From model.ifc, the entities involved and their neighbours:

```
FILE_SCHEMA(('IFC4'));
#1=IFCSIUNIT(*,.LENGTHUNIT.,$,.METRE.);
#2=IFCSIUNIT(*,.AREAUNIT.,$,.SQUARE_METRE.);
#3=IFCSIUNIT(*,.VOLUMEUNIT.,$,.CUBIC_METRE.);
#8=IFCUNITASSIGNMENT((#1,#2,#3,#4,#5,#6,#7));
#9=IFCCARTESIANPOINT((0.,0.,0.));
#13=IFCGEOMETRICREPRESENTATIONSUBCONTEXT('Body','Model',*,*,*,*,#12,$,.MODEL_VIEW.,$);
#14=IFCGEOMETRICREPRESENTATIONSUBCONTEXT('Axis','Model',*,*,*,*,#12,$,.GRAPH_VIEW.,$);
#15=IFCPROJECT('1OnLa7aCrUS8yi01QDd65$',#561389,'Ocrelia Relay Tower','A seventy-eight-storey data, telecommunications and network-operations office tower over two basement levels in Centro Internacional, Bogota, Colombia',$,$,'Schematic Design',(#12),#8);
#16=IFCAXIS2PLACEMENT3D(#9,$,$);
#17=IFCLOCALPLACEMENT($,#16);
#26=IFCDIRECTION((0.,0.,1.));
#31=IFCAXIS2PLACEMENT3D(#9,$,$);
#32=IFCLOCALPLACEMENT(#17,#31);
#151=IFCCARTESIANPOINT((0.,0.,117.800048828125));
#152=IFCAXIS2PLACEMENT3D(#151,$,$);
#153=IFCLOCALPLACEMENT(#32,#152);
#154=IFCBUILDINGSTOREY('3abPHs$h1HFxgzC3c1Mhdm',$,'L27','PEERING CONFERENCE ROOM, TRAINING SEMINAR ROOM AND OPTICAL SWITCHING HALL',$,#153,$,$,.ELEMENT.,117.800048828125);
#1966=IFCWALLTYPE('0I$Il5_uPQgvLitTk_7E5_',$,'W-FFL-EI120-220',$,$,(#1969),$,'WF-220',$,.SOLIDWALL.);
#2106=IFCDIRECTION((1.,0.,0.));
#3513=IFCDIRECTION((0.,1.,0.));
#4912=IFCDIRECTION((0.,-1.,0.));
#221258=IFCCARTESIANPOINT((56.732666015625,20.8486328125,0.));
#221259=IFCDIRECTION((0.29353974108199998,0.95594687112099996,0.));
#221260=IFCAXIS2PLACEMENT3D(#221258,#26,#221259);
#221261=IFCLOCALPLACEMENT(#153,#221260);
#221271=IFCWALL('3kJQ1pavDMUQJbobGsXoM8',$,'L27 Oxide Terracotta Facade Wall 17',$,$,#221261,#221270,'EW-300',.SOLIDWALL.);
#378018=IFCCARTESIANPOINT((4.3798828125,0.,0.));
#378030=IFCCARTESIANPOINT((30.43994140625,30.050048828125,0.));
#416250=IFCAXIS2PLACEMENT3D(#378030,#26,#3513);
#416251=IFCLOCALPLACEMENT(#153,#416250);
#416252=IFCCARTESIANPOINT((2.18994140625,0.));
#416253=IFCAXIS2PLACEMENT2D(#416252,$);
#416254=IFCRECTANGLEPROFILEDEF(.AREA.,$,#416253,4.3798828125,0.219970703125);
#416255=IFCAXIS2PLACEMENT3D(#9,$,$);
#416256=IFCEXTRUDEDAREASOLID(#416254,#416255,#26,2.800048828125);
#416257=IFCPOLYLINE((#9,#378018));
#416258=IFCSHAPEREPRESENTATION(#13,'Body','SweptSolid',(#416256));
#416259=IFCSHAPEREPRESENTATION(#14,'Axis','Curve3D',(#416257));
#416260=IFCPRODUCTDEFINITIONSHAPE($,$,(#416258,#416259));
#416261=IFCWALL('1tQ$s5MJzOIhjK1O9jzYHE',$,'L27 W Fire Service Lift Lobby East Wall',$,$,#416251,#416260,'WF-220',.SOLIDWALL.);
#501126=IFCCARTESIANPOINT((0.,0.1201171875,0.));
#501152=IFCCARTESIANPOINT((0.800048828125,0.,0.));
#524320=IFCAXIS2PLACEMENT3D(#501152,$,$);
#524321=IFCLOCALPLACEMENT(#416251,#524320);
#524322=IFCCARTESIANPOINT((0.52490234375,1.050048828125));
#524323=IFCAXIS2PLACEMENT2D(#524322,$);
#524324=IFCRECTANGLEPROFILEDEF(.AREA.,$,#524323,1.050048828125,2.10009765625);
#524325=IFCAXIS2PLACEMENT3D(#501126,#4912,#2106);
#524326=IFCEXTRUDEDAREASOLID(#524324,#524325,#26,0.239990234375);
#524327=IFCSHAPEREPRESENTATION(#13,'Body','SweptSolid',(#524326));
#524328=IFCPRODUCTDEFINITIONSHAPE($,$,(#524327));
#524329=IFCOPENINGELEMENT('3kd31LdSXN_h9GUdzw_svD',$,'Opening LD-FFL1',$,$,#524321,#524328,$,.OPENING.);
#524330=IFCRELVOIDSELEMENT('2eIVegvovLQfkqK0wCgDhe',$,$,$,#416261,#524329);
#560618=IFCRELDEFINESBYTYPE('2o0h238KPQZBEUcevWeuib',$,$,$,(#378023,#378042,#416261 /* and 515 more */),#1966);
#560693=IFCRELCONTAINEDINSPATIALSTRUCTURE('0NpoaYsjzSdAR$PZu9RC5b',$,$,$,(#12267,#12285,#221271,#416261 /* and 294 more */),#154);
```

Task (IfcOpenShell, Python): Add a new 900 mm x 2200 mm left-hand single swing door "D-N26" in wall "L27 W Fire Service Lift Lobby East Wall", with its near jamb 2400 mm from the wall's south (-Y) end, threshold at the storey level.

```python
import numpy as np
import ifcopenshell
import ifcopenshell.api.feature
import ifcopenshell.api.geometry
import ifcopenshell.api.root
import ifcopenshell.api.spatial
import ifcopenshell.geom
import ifcopenshell.util.element
import ifcopenshell.util.placement
import ifcopenshell.util.representation
import ifcopenshell.util.shape
import ifcopenshell.util.unit

model = ifcopenshell.open("model.ifc")
unit_scale = ifcopenshell.util.unit.calculate_unit_scale(model)
settings = ifcopenshell.geom.settings()


def volume(element):
    """Net volume in cubic metres, openings subtracted."""
    shape = ifcopenshell.geom.create_shape(settings, element)
    return ifcopenshell.util.shape.get_volume(shape.geometry)


wall = model.by_guid("1tQ$s5MJzOIhjK1O9jzYHE")
storey = ifcopenshell.util.element.get_container(wall, ifc_class="IfcBuildingStorey")
context = ifcopenshell.util.representation.get_context(model, "Model", "Body", "MODEL_VIEW")
before = volume(wall)

width, height, from_end, sill = 0.9, 2.2, 2.4, 0.0  # metres

# The wall runs along its own X axis, and the end named is its -X end.
wall_shape = ifcopenshell.geom.create_shape(settings, wall)
x, y, z = ifcopenshell.util.shape.get_vertices(wall_shape.geometry).T
start = x.min() + from_end
face, thickness = float(y.min()), float(y.max() - y.min())
wall_matrix = ifcopenshell.util.placement.get_local_placement(wall.ObjectPlacement)
level = ifcopenshell.util.placement.get_local_placement(storey.ObjectPlacement)[2, 3]


def in_wall(x, y):
    """Placement at x, y metres in the wall's axes, at sill height."""
    matrix = wall_matrix.copy()
    matrix[:, 3] = wall_matrix @ np.array([x / unit_scale, y / unit_scale, 0.0, 1.0])
    matrix[2, 3] = level + sill / unit_scale
    return matrix


# Opening: a box that overshoots both wall faces by 50 mm.
opening = ifcopenshell.api.root.create_entity(model, ifc_class="IfcOpeningElement", predefined_type="OPENING")
box = ifcopenshell.api.geometry.add_wall_representation(
    model, context=context, length=width, height=height, thickness=thickness + 0.1
)
ifcopenshell.api.geometry.assign_representation(model, product=opening, representation=box)
ifcopenshell.api.geometry.edit_object_placement(model, product=opening, matrix=in_wall(start, face - 0.05), is_si=False)
ifcopenshell.api.feature.add_feature(model, feature=opening, element=wall)

door = ifcopenshell.api.root.create_entity(model, ifc_class="IfcDoor", name="D-N26", predefined_type="DOOR")
door.OverallWidth, door.OverallHeight = width / unit_scale, height / unit_scale
door.OperationType = "SINGLE_SWING_LEFT"
body = ifcopenshell.api.geometry.add_door_representation(
    model,
    context=context,
    overall_width=door.OverallWidth,
    overall_height=door.OverallHeight,
    operation_type="SINGLE_SWING_LEFT",
    lining_properties={"LiningDepth": thickness / unit_scale, "ThresholdDepth": thickness / unit_scale},
)
ifcopenshell.api.geometry.assign_representation(model, product=door, representation=body)
ifcopenshell.api.spatial.assign_container(model, products=[door], relating_structure=storey)
ifcopenshell.api.feature.add_filling(model, opening=opening, element=door)

# The lining spans the wall, so the door starts at the wall face.
ifcopenshell.api.geometry.edit_object_placement(model, product=door, matrix=in_wall(start, face), is_si=False)

after = volume(wall)

print(f"wall volume {before:.3f} -> {after:.3f} m3")

model.write("model_v2.ifc")
```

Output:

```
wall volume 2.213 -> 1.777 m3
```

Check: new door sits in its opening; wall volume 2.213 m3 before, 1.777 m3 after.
